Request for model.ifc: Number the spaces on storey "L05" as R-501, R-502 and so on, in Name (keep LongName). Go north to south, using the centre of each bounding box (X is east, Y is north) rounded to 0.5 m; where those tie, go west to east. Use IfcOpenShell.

First a look at what the model holds.

```python
import ifcopenshell
import ifcopenshell.util.element
import ifcopenshell.util.placement

model = ifcopenshell.open("model.ifc")
print(model.schema)
storey = next(s for s in model.by_type("IfcBuildingStorey") if s.Name == "L05")
spaces = [e for e in ifcopenshell.util.element.get_decomposition(storey) if e.is_a("IfcSpace")]
for e in sorted(spaces, key=lambda e: e.id()):
    origin = ifcopenshell.util.placement.get_local_placement(e.ObjectPlacement)[:3, 3]
    print(e.id(), e.Name, e.LongName, origin.round(2) + 0.0, sep=" | ")
```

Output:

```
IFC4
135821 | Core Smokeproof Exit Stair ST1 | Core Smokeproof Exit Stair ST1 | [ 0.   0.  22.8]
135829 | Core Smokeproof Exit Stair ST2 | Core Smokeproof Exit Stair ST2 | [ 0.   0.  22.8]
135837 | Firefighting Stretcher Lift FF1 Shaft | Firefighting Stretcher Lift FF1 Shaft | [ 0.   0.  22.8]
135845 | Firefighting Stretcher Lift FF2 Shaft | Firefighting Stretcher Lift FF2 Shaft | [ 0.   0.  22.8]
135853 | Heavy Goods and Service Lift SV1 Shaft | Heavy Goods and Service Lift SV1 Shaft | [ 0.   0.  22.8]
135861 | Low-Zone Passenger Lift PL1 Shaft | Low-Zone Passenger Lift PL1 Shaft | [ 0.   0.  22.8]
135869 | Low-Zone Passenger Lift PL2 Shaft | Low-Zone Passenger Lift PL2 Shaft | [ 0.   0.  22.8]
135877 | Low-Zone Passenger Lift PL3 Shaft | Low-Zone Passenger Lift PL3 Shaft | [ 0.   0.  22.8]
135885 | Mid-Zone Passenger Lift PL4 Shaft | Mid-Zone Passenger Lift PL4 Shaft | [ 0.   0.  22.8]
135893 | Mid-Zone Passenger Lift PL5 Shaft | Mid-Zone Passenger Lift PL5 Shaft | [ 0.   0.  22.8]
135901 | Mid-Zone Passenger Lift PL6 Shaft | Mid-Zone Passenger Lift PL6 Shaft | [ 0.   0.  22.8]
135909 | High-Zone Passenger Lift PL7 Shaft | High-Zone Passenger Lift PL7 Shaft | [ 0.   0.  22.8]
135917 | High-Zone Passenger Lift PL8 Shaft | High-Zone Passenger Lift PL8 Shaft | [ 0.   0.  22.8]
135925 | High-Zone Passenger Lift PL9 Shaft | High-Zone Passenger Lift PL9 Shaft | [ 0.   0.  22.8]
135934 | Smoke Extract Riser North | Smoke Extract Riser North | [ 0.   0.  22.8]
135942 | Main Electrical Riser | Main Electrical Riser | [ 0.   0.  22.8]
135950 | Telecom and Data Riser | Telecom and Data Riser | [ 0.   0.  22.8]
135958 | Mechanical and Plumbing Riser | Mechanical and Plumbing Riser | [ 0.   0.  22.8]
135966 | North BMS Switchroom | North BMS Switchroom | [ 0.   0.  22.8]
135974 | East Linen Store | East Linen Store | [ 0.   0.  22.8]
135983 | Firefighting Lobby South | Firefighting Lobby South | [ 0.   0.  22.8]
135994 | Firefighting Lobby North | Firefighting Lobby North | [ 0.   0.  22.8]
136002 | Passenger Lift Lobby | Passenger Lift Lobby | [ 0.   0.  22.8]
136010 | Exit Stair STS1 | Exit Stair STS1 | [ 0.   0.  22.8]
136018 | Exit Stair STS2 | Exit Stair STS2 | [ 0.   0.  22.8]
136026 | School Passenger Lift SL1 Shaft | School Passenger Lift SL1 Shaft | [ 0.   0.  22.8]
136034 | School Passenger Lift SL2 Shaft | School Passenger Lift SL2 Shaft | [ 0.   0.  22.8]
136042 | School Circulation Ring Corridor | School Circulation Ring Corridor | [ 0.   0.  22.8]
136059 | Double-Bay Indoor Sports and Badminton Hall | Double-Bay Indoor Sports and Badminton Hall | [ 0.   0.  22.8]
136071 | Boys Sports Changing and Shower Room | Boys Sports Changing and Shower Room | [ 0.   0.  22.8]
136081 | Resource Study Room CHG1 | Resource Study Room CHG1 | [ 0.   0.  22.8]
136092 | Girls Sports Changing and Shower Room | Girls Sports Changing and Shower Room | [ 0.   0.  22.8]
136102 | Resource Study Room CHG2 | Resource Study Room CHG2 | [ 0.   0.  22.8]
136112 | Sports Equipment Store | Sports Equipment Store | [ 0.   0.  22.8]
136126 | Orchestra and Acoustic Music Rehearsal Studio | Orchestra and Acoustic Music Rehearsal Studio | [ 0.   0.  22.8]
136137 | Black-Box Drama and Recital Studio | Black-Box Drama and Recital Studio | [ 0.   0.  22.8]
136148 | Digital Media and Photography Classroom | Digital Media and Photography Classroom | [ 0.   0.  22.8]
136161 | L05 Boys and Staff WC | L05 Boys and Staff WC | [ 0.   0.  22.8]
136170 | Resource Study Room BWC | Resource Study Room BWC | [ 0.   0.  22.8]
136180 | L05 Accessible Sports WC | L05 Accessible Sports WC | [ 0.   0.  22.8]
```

```python
import ifcopenshell
import ifcopenshell.geom
import ifcopenshell.util.element
import ifcopenshell.util.shape

model = ifcopenshell.open("model.ifc")
settings = ifcopenshell.geom.settings()
settings.set("use-world-coords", True)


def centre(element):
    shape = ifcopenshell.geom.create_shape(settings, element)
    return ifcopenshell.util.shape.get_bbox_centroid(shape.geometry)


storey = next(s for s in model.by_type("IfcBuildingStorey") if s.Name == "L05")
spaces = [e for e in ifcopenshell.util.element.get_decomposition(storey) if e.is_a("IfcSpace")]

# Insertion points can sit at a corner or the storey origin, so sort by the geometry (in metres).
centres = {e: centre(e) for e in spaces}
spaces.sort(key=lambda e: (-round(centres[e][1] / 0.5), centres[e][0]))

for i, e in enumerate(spaces, start=1):
    number = f"R-5{i:02d}"
    e.Name = number
    print(e.id(), number)

model.write("model_v2.ifc")
```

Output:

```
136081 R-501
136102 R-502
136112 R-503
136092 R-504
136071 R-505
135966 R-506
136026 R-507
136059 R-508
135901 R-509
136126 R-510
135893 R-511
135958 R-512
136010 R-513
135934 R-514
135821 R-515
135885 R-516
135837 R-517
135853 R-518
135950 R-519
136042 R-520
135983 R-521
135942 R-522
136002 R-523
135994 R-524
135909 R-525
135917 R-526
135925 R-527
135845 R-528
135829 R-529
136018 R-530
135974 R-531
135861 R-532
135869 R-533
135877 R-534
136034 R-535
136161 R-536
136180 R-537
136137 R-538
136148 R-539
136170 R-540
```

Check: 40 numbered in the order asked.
